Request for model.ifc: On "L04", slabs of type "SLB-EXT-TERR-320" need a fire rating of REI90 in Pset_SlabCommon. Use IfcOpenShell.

First a look at what the model holds.

```python
import ifcopenshell
import ifcopenshell.util.element

model = ifcopenshell.open("model.ifc")
print(model.schema)
storey = next(s for s in model.by_type("IfcBuildingStorey") if s.Name == "L04")
slabs = [e for e in ifcopenshell.util.element.get_decomposition(storey) if e.is_a("IfcSlab")]
seen = {}
for e in slabs:
    element_type = ifcopenshell.util.element.get_type(e)
    key = (element_type.Name if element_type != e and element_type else None, ifcopenshell.util.element.get_pset(e, "Pset_SlabCommon", "FireRating"))
    seen[key] = seen.get(key, 0) + 1
for (name, value), count in sorted(seen.items(), key=str):
    print(count, "x", name, "|", value)
```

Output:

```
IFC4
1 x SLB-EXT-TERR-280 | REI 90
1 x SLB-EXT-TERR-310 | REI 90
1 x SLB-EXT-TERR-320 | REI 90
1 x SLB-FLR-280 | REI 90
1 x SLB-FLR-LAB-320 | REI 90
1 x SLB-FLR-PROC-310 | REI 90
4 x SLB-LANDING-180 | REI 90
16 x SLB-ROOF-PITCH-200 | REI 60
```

```python
import ifcopenshell
import ifcopenshell.api.pset
import ifcopenshell.util.element

model = ifcopenshell.open("model.ifc")

storey = next(s for s in model.by_type("IfcBuildingStorey") if s.Name == "L04")
slabs = [e for e in ifcopenshell.util.element.get_decomposition(storey) if e.is_a("IfcSlab")]

count = 0
for e in slabs:
    element_type = ifcopenshell.util.element.get_type(e)
    if element_type in (None, e) or element_type.Name != "SLB-EXT-TERR-320":
        continue
    # add_pset returns the element's existing set when there is one.
    pset = ifcopenshell.api.pset.add_pset(model, product=e, name="Pset_SlabCommon")
    ifcopenshell.api.pset.edit_pset(model, pset=pset, properties={"FireRating": "REI90"})
    count += 1

print(count, "slabs updated")

model.write("model_updated.ifc")
```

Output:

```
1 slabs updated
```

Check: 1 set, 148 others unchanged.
